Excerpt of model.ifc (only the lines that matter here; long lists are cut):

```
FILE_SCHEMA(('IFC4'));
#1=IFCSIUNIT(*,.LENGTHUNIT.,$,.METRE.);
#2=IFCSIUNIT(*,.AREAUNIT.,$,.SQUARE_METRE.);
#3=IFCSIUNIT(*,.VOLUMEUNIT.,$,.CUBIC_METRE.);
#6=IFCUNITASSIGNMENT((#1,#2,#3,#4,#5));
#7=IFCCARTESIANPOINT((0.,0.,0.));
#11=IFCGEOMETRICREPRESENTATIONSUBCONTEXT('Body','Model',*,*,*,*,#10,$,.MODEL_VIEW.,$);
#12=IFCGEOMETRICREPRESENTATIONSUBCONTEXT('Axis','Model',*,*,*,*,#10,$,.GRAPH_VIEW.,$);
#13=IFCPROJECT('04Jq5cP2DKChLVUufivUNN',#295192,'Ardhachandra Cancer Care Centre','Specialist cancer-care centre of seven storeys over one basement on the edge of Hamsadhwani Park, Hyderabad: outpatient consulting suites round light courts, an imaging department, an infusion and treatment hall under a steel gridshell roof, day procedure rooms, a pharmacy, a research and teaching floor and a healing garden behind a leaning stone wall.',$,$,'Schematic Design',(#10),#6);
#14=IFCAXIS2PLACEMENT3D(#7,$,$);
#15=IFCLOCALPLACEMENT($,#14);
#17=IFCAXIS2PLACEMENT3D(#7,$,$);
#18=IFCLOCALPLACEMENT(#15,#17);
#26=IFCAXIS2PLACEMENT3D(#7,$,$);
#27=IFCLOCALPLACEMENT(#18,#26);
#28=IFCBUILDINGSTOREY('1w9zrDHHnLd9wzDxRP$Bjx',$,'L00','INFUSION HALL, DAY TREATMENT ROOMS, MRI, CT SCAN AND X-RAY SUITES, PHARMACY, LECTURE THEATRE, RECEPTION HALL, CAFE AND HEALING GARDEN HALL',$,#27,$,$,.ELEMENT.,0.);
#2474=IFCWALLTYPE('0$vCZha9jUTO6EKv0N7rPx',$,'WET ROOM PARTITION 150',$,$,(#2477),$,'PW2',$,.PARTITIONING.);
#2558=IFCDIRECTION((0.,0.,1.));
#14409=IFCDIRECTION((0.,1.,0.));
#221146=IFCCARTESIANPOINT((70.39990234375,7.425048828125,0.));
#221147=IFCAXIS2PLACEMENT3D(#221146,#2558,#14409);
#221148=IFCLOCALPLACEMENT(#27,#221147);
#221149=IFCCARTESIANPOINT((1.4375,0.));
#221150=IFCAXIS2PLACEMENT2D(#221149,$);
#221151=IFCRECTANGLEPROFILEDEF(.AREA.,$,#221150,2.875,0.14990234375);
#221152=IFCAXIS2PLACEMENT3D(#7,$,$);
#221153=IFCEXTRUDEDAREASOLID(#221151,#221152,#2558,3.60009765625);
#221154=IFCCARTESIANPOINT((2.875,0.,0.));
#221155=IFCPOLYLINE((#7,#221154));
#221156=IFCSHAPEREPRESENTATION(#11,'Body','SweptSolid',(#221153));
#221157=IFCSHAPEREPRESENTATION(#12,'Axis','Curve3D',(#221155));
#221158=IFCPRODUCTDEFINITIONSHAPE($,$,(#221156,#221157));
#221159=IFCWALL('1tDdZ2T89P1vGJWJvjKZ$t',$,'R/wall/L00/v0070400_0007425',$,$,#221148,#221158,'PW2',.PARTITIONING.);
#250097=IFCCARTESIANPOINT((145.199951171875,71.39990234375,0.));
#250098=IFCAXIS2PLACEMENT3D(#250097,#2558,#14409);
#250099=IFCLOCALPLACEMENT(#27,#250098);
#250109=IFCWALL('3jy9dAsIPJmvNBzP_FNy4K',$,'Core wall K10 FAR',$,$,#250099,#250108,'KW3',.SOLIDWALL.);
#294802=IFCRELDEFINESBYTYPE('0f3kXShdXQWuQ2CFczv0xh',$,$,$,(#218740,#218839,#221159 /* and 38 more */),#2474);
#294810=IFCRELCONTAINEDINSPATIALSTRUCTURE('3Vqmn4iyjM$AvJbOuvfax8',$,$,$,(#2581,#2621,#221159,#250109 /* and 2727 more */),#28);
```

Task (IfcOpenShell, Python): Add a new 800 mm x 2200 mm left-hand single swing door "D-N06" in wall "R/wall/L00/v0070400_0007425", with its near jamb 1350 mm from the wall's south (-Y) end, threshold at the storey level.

```python
import numpy as np
import ifcopenshell
import ifcopenshell.api.feature
import ifcopenshell.api.geometry
import ifcopenshell.api.root
import ifcopenshell.api.spatial
import ifcopenshell.geom
import ifcopenshell.util.element
import ifcopenshell.util.placement
import ifcopenshell.util.representation
import ifcopenshell.util.shape
import ifcopenshell.util.unit

model = ifcopenshell.open("model.ifc")
unit_scale = ifcopenshell.util.unit.calculate_unit_scale(model)
settings = ifcopenshell.geom.settings()


def volume(element):
    """Net volume in cubic metres, openings subtracted."""
    shape = ifcopenshell.geom.create_shape(settings, element)
    return ifcopenshell.util.shape.get_volume(shape.geometry)


wall = model.by_id(221159)
storey = ifcopenshell.util.element.get_container(wall, ifc_class="IfcBuildingStorey")
context = ifcopenshell.util.representation.get_context(model, "Model", "Body", "MODEL_VIEW")
before = volume(wall)

width, height, from_end, sill = 0.8, 2.2, 1.35, 0.0  # metres

# The wall runs along its own X axis, and the end named is its -X end.
wall_shape = ifcopenshell.geom.create_shape(settings, wall)
x, y, z = ifcopenshell.util.shape.get_vertices(wall_shape.geometry).T
start = x.min() + from_end
face, thickness = float(y.min()), float(y.max() - y.min())
wall_matrix = ifcopenshell.util.placement.get_local_placement(wall.ObjectPlacement)
level = ifcopenshell.util.placement.get_local_placement(storey.ObjectPlacement)[2, 3]


def in_wall(x, y):
    """Placement at x, y metres in the wall's axes, at sill height."""
    matrix = wall_matrix.copy()
    matrix[:, 3] = wall_matrix @ np.array([x / unit_scale, y / unit_scale, 0.0, 1.0])
    matrix[2, 3] = level + sill / unit_scale
    return matrix


# Opening: a box that overshoots both wall faces by 50 mm.
opening = ifcopenshell.api.root.create_entity(model, ifc_class="IfcOpeningElement", predefined_type="OPENING")
box = ifcopenshell.api.geometry.add_wall_representation(
    model, context=context, length=width, height=height, thickness=thickness + 0.1
)
ifcopenshell.api.geometry.assign_representation(model, product=opening, representation=box)
ifcopenshell.api.geometry.edit_object_placement(model, product=opening, matrix=in_wall(start, face - 0.05), is_si=False)
ifcopenshell.api.feature.add_feature(model, feature=opening, element=wall)

door = ifcopenshell.api.root.create_entity(model, ifc_class="IfcDoor", name="D-N06", predefined_type="DOOR")
door.OverallWidth, door.OverallHeight = width / unit_scale, height / unit_scale
door.OperationType = "SINGLE_SWING_LEFT"
body = ifcopenshell.api.geometry.add_door_representation(
    model,
    context=context,
    overall_width=door.OverallWidth,
    overall_height=door.OverallHeight,
    operation_type="SINGLE_SWING_LEFT",
    lining_properties={"LiningDepth": thickness / unit_scale, "ThresholdDepth": thickness / unit_scale},
)
ifcopenshell.api.geometry.assign_representation(model, product=door, representation=body)
ifcopenshell.api.spatial.assign_container(model, products=[door], relating_structure=storey)
ifcopenshell.api.feature.add_filling(model, opening=opening, element=door)

# The lining spans the wall, so the door starts at the wall face.
ifcopenshell.api.geometry.edit_object_placement(model, product=door, matrix=in_wall(start, face), is_si=False)

after = volume(wall)

print(f"wall volume {before:.3f} -> {after:.3f} m3")

model.write("model_v2.ifc")
```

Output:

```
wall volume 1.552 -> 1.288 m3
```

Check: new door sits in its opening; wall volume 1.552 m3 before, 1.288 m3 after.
